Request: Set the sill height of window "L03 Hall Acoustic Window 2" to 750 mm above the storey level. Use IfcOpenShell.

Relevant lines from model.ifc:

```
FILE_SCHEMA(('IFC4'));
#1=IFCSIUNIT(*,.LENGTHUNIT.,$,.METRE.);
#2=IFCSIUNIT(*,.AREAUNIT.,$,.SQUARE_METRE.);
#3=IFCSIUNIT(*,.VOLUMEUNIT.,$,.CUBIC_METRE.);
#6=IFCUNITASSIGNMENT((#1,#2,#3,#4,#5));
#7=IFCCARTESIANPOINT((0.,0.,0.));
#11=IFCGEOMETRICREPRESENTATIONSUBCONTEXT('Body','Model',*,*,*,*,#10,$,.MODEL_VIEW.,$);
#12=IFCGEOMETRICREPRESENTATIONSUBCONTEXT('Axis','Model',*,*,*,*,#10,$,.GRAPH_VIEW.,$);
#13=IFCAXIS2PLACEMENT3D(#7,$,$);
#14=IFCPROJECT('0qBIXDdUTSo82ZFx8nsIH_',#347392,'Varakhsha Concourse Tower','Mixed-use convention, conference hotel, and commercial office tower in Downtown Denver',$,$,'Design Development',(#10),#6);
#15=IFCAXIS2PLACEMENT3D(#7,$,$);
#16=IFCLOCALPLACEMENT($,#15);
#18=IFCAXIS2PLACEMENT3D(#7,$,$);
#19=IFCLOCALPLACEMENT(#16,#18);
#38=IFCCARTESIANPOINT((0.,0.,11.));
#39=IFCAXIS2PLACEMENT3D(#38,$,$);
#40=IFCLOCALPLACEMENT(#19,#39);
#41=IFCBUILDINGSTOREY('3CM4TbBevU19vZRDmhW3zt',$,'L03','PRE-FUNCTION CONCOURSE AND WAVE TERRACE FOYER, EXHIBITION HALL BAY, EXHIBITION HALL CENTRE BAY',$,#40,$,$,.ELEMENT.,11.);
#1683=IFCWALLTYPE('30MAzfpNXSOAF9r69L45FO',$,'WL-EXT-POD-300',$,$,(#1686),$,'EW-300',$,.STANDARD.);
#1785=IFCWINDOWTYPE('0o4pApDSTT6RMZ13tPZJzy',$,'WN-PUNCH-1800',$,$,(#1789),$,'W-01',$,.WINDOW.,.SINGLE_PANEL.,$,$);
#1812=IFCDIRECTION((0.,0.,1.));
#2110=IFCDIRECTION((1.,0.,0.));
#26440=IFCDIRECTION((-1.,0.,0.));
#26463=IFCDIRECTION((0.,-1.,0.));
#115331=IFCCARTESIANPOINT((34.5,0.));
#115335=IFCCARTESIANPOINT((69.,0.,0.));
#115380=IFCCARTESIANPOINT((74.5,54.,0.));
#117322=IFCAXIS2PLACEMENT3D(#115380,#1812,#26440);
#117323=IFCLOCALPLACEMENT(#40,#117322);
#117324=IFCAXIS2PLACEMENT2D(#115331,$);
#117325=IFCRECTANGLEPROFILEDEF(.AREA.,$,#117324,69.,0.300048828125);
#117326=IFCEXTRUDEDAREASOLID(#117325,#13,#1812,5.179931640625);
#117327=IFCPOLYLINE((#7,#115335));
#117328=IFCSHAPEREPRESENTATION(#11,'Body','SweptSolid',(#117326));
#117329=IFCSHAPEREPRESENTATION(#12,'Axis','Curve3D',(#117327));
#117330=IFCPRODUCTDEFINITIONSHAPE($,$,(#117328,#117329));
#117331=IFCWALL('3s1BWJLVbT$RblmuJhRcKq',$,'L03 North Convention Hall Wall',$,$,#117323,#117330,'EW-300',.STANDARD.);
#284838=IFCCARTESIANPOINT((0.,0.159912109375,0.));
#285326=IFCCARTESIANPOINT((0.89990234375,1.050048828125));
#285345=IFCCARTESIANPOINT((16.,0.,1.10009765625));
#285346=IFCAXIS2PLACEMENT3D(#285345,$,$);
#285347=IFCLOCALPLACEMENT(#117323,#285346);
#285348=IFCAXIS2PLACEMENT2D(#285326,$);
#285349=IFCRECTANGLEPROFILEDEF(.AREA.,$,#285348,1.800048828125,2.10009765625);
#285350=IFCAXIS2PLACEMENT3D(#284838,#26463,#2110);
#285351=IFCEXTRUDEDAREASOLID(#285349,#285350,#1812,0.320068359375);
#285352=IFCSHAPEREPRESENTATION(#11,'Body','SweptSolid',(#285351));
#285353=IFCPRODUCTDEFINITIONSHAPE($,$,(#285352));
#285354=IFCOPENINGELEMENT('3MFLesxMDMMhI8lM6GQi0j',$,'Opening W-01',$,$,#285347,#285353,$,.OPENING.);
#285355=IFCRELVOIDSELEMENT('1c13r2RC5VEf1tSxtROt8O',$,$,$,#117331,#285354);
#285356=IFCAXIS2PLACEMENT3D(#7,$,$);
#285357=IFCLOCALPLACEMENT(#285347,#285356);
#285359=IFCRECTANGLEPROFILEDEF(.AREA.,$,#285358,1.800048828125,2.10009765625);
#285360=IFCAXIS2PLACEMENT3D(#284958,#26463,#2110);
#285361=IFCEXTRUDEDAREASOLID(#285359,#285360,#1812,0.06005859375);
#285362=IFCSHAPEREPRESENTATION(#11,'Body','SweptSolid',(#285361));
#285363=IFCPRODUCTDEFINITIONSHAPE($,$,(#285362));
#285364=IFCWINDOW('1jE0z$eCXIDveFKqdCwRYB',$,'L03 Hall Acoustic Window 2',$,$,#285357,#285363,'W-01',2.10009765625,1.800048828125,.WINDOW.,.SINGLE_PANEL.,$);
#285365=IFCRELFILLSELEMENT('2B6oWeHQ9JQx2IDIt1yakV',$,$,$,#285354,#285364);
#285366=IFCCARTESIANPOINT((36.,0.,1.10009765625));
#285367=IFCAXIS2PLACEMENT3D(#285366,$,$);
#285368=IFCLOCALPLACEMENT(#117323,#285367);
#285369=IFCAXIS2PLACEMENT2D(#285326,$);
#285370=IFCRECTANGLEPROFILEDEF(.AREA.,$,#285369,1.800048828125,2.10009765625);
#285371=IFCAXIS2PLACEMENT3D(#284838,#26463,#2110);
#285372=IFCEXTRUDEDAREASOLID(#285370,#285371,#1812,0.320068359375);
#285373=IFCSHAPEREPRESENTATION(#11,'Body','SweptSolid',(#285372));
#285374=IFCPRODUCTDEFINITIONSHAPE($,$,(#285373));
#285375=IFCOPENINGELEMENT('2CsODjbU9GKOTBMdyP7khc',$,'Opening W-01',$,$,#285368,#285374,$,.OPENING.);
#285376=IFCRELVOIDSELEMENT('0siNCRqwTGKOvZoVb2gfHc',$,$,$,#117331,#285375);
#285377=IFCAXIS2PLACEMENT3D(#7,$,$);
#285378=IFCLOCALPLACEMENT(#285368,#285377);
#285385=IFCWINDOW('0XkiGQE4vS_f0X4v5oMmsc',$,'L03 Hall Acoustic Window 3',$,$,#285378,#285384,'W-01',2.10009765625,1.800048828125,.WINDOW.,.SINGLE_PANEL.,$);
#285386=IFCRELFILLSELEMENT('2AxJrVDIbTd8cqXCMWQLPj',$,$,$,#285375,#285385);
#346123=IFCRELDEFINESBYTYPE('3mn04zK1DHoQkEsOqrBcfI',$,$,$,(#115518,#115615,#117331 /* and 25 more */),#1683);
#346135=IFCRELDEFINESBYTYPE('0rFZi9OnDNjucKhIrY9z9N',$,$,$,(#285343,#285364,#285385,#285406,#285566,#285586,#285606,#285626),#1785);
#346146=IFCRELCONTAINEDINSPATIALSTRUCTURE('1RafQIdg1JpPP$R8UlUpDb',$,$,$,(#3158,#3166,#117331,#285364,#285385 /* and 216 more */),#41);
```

```python
import numpy as np
import ifcopenshell
import ifcopenshell.api.geometry
import ifcopenshell.geom
import ifcopenshell.util.element
import ifcopenshell.util.placement
import ifcopenshell.util.shape
import ifcopenshell.util.unit

model = ifcopenshell.open("model.ifc")
unit_scale = ifcopenshell.util.unit.calculate_unit_scale(model)

window = model.by_guid("1jE0z$eCXIDveFKqdCwRYB")
opening = window.FillsVoids[0].RelatingOpeningElement
storey = ifcopenshell.util.element.get_container(window, ifc_class="IfcBuildingStorey")
level = ifcopenshell.util.placement.get_local_placement(storey.ObjectPlacement)[2, 3]

# The opening's origin need not be at the sill, so measure its lowest point.
shape = ifcopenshell.geom.create_shape(ifcopenshell.geom.settings(), opening)
bottom = ifcopenshell.util.shape.get_shape_bottom_elevation(shape, shape.geometry) / unit_scale
dz = level + 0.75 - bottom

shift = np.array([0.0, 0.0, dz])
# The window is placed relative to its opening, so it follows when the opening moves.
matrix = ifcopenshell.util.placement.get_local_placement(opening.ObjectPlacement)
matrix[:3, 3] += shift
ifcopenshell.api.geometry.edit_object_placement(
    model, product=opening, matrix=matrix, is_si=False, should_transform_children=True
)

print(f"moved by {dz * unit_scale:+.3f} m")

model.write("model_updated.ifc")
```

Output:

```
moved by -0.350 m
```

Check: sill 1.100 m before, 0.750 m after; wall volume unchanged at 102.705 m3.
